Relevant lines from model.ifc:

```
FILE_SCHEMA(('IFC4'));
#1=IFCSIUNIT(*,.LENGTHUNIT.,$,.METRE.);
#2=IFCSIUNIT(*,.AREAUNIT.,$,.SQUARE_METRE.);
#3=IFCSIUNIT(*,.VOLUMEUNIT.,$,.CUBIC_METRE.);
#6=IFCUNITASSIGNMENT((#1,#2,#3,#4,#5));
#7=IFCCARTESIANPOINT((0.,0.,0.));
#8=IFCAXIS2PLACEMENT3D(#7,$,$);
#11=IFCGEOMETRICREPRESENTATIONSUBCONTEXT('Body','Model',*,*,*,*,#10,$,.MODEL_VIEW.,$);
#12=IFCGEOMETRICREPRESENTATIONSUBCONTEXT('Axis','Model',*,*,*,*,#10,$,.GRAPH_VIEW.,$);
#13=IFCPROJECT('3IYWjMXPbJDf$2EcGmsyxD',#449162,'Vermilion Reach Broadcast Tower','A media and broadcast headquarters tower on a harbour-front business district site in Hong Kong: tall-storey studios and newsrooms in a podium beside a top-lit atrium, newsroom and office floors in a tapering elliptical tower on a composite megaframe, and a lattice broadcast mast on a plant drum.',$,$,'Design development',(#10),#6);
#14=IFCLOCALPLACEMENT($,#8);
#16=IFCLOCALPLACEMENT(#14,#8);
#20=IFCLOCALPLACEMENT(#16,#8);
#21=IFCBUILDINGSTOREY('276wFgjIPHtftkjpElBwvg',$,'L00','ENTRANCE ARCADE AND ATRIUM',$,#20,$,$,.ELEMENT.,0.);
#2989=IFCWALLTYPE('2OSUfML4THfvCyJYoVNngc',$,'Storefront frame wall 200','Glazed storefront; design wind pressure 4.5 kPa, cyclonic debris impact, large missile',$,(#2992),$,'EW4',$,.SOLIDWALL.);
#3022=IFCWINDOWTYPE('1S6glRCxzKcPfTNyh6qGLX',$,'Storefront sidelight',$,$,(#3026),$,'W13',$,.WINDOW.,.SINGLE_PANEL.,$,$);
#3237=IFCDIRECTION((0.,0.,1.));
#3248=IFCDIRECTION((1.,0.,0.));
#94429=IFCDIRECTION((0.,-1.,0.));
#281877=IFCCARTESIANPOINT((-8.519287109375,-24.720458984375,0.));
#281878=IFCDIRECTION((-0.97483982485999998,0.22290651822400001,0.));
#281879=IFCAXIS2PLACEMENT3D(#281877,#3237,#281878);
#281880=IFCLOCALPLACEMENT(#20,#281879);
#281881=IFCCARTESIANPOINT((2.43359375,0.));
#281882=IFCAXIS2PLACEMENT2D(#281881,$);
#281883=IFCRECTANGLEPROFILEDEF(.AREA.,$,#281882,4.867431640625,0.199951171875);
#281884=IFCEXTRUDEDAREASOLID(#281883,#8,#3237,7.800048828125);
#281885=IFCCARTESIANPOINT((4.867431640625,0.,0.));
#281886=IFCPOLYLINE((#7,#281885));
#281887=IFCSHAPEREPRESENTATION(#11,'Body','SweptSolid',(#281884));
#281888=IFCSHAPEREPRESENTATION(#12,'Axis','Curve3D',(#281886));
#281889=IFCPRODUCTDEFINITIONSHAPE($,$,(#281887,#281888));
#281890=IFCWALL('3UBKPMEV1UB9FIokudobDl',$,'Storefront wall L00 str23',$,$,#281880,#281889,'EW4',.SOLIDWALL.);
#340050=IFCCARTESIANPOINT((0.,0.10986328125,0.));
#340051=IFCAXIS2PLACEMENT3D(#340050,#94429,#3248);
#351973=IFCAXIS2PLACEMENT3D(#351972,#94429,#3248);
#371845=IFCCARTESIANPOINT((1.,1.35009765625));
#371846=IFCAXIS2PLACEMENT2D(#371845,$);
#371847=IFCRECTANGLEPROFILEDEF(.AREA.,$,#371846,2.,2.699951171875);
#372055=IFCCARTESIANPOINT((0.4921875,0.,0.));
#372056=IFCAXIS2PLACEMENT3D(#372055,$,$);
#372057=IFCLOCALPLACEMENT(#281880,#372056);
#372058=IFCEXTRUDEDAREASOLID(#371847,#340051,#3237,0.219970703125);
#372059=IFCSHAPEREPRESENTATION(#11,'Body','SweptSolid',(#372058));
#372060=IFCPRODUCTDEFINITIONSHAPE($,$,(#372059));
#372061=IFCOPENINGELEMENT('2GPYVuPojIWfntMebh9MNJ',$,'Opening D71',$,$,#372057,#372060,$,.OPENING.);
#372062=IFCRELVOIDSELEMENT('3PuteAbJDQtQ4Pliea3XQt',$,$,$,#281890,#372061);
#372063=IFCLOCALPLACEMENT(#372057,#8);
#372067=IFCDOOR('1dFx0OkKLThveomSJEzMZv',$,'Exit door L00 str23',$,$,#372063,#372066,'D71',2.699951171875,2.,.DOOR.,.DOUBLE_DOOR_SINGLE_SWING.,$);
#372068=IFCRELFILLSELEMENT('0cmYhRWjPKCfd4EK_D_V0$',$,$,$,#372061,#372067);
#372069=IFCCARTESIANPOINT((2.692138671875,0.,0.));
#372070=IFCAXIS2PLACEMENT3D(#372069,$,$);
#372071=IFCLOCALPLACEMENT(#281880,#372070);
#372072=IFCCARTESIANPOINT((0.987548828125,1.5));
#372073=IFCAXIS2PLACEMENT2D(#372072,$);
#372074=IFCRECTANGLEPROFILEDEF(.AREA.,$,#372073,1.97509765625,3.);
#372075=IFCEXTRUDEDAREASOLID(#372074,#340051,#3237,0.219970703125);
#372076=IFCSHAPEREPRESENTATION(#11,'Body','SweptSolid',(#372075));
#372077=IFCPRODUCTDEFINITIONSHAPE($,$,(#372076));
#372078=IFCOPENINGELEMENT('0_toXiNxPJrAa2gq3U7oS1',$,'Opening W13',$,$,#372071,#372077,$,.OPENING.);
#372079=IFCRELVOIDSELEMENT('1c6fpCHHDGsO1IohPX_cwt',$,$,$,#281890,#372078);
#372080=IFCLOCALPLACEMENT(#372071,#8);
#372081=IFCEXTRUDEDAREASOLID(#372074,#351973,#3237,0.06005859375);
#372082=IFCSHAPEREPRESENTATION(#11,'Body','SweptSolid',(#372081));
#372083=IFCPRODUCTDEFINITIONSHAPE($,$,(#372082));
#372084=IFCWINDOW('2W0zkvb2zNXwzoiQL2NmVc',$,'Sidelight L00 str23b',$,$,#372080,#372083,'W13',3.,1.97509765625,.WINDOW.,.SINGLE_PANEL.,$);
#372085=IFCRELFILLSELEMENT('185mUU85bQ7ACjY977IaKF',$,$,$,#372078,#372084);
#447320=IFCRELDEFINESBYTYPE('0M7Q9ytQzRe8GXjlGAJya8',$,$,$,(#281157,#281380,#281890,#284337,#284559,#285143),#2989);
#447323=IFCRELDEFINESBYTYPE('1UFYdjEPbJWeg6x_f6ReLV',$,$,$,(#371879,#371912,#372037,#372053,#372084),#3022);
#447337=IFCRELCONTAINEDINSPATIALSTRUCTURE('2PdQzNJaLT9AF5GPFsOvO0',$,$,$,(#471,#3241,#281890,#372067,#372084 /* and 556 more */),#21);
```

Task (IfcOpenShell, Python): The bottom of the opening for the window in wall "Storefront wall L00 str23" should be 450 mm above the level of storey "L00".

```python
import numpy as np
import ifcopenshell
import ifcopenshell.api.geometry
import ifcopenshell.geom
import ifcopenshell.util.element
import ifcopenshell.util.placement
import ifcopenshell.util.shape
import ifcopenshell.util.unit

model = ifcopenshell.open("model.ifc")
unit_scale = ifcopenshell.util.unit.calculate_unit_scale(model)

window = model.by_id(372084)
opening = window.FillsVoids[0].RelatingOpeningElement
storey = ifcopenshell.util.element.get_container(window, ifc_class="IfcBuildingStorey")
level = ifcopenshell.util.placement.get_local_placement(storey.ObjectPlacement)[2, 3]

# The opening's origin need not be at the sill, so measure its lowest point.
shape = ifcopenshell.geom.create_shape(ifcopenshell.geom.settings(), opening)
bottom = ifcopenshell.util.shape.get_shape_bottom_elevation(shape, shape.geometry) / unit_scale
dz = level + 0.45 / unit_scale - bottom

shift = np.array([0.0, 0.0, dz])
# The window is placed relative to its opening, so it follows when the opening moves.
matrix = ifcopenshell.util.placement.get_local_placement(opening.ObjectPlacement)
matrix[:3, 3] += shift
ifcopenshell.api.geometry.edit_object_placement(
    model, product=opening, matrix=matrix, is_si=False, should_transform_children=True
)

print(f"moved by {dz * unit_scale:+.3f} m")

model.write("model_v2.ifc")
```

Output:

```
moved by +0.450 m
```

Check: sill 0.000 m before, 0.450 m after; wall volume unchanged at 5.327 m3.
